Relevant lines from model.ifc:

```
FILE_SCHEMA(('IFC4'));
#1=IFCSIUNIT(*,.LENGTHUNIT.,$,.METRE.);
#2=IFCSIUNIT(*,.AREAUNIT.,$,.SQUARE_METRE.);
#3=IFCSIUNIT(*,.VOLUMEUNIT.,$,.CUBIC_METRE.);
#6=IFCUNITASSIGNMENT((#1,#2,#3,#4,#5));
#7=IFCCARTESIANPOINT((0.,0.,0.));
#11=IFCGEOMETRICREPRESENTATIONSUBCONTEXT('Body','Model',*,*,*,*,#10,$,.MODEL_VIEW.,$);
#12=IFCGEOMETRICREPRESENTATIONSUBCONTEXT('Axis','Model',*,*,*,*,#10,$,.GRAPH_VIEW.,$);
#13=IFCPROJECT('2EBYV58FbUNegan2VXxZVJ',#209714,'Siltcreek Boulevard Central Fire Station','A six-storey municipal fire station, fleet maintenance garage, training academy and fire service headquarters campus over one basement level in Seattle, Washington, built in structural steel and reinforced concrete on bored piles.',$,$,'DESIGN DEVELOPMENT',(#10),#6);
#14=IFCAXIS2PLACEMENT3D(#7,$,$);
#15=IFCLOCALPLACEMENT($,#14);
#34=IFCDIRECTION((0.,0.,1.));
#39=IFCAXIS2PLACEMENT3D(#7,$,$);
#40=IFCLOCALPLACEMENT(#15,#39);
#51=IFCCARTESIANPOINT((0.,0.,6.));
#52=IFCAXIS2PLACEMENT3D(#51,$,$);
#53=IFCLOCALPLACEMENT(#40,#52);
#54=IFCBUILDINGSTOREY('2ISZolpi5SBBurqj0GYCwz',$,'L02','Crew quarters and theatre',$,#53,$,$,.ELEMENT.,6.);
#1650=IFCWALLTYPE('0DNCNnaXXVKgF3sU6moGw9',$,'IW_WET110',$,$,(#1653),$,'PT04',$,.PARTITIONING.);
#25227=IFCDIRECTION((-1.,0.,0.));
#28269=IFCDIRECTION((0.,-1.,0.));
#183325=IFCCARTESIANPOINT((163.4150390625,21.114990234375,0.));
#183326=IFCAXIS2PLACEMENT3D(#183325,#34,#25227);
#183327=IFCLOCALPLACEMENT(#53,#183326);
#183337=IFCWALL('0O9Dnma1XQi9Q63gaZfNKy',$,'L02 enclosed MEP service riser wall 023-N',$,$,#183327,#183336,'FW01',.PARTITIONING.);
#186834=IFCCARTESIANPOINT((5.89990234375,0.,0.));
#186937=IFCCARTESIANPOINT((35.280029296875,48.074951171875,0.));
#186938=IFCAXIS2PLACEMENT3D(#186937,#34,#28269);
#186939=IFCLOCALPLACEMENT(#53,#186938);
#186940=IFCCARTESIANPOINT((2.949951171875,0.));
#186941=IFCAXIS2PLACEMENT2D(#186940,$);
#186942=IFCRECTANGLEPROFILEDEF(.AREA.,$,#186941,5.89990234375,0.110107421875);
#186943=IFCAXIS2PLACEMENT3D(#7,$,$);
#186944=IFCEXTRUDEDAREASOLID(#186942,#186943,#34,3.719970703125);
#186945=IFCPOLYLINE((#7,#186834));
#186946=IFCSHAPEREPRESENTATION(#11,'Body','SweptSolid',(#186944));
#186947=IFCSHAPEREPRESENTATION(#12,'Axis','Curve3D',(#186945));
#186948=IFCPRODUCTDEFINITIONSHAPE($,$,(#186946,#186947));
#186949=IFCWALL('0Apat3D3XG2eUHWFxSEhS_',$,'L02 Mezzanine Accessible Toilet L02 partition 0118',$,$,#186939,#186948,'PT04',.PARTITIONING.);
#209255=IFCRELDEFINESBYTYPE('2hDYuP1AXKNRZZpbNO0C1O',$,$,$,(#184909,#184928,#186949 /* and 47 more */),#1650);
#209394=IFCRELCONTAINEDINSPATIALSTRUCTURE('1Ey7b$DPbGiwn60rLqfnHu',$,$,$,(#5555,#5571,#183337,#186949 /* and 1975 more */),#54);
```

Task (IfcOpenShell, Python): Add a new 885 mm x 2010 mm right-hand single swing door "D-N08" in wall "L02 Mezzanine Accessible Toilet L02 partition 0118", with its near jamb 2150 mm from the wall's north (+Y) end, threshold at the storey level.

```python
import numpy as np
import ifcopenshell
import ifcopenshell.api.feature
import ifcopenshell.api.geometry
import ifcopenshell.api.root
import ifcopenshell.api.spatial
import ifcopenshell.geom
import ifcopenshell.util.element
import ifcopenshell.util.placement
import ifcopenshell.util.representation
import ifcopenshell.util.shape
import ifcopenshell.util.unit

model = ifcopenshell.open("model.ifc")
unit_scale = ifcopenshell.util.unit.calculate_unit_scale(model)
settings = ifcopenshell.geom.settings()


def volume(element):
    """Net volume in cubic metres, openings subtracted."""
    shape = ifcopenshell.geom.create_shape(settings, element)
    return ifcopenshell.util.shape.get_volume(shape.geometry)


wall = model.by_guid("0Apat3D3XG2eUHWFxSEhS_")
storey = ifcopenshell.util.element.get_container(wall, ifc_class="IfcBuildingStorey")
context = ifcopenshell.util.representation.get_context(model, "Model", "Body", "MODEL_VIEW")
before = volume(wall)

width, height, from_end, sill = 0.885, 2.01, 2.15, 0.0  # metres

# The wall runs along its own X axis, and the end named is its -X end.
wall_shape = ifcopenshell.geom.create_shape(settings, wall)
x, y, z = ifcopenshell.util.shape.get_vertices(wall_shape.geometry).T
start = x.min() + from_end
face, thickness = float(y.min()), float(y.max() - y.min())
wall_matrix = ifcopenshell.util.placement.get_local_placement(wall.ObjectPlacement)
level = ifcopenshell.util.placement.get_local_placement(storey.ObjectPlacement)[2, 3]


def in_wall(x, y):
    """Placement at x, y metres in the wall's axes, at sill height."""
    matrix = wall_matrix.copy()
    matrix[:, 3] = wall_matrix @ np.array([x / unit_scale, y / unit_scale, 0.0, 1.0])
    matrix[2, 3] = level + sill / unit_scale
    return matrix


# Opening: a box that overshoots both wall faces by 50 mm.
opening = ifcopenshell.api.root.create_entity(model, ifc_class="IfcOpeningElement", predefined_type="OPENING")
box = ifcopenshell.api.geometry.add_wall_representation(
    model, context=context, length=width, height=height, thickness=thickness + 0.1
)
ifcopenshell.api.geometry.assign_representation(model, product=opening, representation=box)
ifcopenshell.api.geometry.edit_object_placement(model, product=opening, matrix=in_wall(start, face - 0.05), is_si=False)
ifcopenshell.api.feature.add_feature(model, feature=opening, element=wall)

door = ifcopenshell.api.root.create_entity(model, ifc_class="IfcDoor", name="D-N08", predefined_type="DOOR")
door.OverallWidth, door.OverallHeight = width / unit_scale, height / unit_scale
door.OperationType = "SINGLE_SWING_RIGHT"
body = ifcopenshell.api.geometry.add_door_representation(
    model,
    context=context,
    overall_width=door.OverallWidth,
    overall_height=door.OverallHeight,
    operation_type="SINGLE_SWING_RIGHT",
    lining_properties={"LiningDepth": thickness / unit_scale, "ThresholdDepth": thickness / unit_scale},
)
ifcopenshell.api.geometry.assign_representation(model, product=door, representation=body)
ifcopenshell.api.spatial.assign_container(model, products=[door], relating_structure=storey)
ifcopenshell.api.feature.add_filling(model, opening=opening, element=door)

# The lining spans the wall, so the door starts at the wall face.
ifcopenshell.api.geometry.edit_object_placement(model, product=door, matrix=in_wall(start, face), is_si=False)

after = volume(wall)

print(f"wall volume {before:.3f} -> {after:.3f} m3")

model.write("model-out.ifc")
```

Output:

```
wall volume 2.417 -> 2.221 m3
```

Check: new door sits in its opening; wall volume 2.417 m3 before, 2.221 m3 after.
